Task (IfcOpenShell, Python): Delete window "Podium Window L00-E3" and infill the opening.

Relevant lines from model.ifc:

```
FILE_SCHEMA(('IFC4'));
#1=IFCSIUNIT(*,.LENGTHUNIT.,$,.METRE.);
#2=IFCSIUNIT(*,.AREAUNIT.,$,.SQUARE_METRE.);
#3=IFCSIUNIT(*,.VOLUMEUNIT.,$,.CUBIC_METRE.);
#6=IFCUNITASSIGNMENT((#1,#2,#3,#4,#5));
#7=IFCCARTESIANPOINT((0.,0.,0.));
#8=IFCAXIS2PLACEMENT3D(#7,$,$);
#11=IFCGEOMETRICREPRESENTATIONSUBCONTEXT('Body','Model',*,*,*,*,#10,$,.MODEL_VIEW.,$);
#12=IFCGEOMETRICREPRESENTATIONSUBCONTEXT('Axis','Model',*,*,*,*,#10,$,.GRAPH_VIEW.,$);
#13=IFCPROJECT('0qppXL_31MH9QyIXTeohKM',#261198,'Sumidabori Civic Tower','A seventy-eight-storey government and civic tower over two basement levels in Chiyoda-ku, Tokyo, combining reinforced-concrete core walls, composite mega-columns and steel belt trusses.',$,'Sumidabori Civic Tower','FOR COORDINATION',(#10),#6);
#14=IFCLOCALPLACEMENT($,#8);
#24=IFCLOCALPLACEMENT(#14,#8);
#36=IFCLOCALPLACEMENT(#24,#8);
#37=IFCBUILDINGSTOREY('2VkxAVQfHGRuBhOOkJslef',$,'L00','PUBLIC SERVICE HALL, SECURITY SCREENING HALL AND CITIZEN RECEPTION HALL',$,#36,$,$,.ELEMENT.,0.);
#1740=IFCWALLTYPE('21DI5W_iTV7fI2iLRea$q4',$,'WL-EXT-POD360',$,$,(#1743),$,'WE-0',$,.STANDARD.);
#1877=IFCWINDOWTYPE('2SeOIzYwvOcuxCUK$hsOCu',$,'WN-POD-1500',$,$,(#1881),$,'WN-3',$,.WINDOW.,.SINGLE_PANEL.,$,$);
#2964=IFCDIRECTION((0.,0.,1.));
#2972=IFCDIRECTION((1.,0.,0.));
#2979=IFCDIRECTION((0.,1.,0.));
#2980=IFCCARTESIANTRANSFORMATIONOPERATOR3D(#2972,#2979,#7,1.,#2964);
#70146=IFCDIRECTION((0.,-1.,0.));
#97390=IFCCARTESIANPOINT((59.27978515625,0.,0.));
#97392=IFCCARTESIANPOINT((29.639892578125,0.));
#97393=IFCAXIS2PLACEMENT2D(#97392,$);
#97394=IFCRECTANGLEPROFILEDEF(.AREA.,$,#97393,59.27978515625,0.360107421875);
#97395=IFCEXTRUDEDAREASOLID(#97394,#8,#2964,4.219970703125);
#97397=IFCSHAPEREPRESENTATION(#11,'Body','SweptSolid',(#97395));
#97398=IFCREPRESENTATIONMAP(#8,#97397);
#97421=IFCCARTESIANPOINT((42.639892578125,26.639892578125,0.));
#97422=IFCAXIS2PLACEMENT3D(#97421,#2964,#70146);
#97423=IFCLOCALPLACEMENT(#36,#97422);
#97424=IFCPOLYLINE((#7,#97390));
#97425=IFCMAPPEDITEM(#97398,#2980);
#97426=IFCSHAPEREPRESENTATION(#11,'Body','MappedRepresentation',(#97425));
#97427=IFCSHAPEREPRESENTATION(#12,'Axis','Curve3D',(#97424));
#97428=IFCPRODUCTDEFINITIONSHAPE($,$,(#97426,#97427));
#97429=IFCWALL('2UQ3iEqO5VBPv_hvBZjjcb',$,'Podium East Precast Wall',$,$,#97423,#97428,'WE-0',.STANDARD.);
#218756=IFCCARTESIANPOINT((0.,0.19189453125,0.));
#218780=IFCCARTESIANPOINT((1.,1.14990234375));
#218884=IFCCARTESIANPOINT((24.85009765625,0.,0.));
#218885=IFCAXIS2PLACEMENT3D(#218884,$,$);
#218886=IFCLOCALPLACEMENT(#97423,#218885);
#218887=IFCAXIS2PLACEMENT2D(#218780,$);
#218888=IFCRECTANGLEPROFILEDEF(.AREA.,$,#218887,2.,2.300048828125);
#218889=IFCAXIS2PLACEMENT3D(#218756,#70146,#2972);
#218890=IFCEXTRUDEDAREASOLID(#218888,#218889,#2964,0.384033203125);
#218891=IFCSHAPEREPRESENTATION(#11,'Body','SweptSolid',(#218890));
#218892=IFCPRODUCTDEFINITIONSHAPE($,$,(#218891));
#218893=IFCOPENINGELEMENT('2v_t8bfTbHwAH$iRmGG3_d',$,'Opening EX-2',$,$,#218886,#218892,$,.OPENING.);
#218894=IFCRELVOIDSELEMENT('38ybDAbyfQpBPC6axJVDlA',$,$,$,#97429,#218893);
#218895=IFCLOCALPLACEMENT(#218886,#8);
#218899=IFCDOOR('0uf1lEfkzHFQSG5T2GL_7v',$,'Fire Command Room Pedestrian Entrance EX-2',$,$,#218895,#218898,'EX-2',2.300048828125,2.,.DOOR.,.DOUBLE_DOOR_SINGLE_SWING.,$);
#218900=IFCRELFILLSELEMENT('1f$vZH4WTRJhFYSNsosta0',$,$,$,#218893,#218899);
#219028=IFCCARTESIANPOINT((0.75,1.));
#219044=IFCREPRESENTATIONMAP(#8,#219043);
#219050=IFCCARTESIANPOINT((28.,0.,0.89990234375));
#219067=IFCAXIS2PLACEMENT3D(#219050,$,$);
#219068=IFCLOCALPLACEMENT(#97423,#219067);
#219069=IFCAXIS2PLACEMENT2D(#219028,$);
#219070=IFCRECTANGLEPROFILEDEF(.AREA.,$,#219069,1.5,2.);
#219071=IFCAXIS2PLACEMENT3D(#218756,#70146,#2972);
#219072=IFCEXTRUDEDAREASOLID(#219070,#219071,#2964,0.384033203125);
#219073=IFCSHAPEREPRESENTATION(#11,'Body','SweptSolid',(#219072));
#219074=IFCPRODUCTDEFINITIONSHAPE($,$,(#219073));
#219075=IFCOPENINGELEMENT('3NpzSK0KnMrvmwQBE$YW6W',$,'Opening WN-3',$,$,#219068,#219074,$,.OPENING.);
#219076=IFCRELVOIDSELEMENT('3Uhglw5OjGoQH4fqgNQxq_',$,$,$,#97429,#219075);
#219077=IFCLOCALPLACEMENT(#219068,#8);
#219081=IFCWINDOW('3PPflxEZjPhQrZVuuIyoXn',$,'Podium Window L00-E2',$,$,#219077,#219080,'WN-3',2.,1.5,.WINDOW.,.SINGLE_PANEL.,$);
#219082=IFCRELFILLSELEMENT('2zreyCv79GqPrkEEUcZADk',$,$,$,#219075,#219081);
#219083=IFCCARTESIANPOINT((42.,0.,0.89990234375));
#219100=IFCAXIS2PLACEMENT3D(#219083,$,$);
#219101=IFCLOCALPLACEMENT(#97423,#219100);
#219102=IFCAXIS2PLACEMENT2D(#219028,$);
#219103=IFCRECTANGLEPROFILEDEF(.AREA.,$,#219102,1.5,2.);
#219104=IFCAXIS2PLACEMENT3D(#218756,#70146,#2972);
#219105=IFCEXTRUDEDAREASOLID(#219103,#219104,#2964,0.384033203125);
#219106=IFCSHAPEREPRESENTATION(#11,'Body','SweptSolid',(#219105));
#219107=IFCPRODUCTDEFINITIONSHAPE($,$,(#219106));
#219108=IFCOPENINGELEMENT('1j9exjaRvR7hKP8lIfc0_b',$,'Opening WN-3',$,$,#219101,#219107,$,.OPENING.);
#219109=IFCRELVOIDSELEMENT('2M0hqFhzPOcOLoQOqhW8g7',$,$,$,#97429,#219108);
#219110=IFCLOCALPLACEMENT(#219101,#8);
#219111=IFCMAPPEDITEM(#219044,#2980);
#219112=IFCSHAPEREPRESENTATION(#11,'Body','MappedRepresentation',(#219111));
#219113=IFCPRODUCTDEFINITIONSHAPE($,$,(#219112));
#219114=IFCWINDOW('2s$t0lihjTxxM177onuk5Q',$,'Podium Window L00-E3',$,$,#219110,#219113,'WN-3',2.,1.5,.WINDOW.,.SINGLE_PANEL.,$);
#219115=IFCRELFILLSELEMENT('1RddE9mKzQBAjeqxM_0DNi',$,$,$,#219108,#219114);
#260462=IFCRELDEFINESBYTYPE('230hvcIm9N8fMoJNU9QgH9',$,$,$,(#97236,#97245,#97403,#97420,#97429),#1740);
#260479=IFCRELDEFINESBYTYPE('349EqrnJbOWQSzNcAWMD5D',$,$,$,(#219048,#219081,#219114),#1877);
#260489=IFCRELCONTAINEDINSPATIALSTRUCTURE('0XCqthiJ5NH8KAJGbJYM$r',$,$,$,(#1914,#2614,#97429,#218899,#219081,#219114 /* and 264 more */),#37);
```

```python
import ifcopenshell
import ifcopenshell.api.feature
import ifcopenshell.api.root
import ifcopenshell.geom
import ifcopenshell.util.shape

model = ifcopenshell.open("model.ifc")
settings = ifcopenshell.geom.settings()


def volume(element):
    """Net volume in cubic metres, openings subtracted."""
    shape = ifcopenshell.geom.create_shape(settings, element)
    return ifcopenshell.util.shape.get_volume(shape.geometry)


window = model.by_guid("2s$t0lihjTxxM177onuk5Q")
opening = window.FillsVoids[0].RelatingOpeningElement
wall = opening.VoidsElements[0].RelatingBuildingElement
before = volume(wall)

ifcopenshell.api.root.remove_product(model, product=window)
ifcopenshell.api.feature.remove_feature(model, feature=opening)

after = volume(wall)

print(f"wall volume {before:.3f} -> {after:.3f} m3")

model.write("model-out.ifc")
```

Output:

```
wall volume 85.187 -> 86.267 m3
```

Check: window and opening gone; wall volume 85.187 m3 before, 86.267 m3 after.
